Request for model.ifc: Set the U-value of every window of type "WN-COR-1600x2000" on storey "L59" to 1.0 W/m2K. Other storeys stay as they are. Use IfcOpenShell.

First a look at what the model holds.

```python
import ifcopenshell
import ifcopenshell.util.element

model = ifcopenshell.open("model.ifc")
print(model.schema)
storey = next(s for s in model.by_type("IfcBuildingStorey") if s.Name == "L59")
windows = [e for e in ifcopenshell.util.element.get_decomposition(storey) if e.is_a("IfcWindow")]
seen = {}
for e in windows:
    element_type = ifcopenshell.util.element.get_type(e)
    key = (element_type.Name if element_type != e and element_type else None, ifcopenshell.util.element.get_pset(e, "Pset_WindowCommon", "ThermalTransmittance"))
    seen[key] = seen.get(key, 0) + 1
for (name, value), count in sorted(seen.items(), key=str):
    print(count, "x", name, "|", value)
```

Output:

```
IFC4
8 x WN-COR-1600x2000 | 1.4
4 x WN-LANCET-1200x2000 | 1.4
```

```python
import ifcopenshell
import ifcopenshell.api.pset
import ifcopenshell.util.element

model = ifcopenshell.open("model.ifc")

storey = next(s for s in model.by_type("IfcBuildingStorey") if s.Name == "L59")
windows = [e for e in ifcopenshell.util.element.get_decomposition(storey) if e.is_a("IfcWindow")]

count = 0
for e in windows:
    element_type = ifcopenshell.util.element.get_type(e)
    if element_type in (None, e) or element_type.Name != "WN-COR-1600x2000":
        continue
    found = ifcopenshell.util.element.get_pset(e, "Pset_WindowCommon", should_inherit=False)
    if found:
        pset = model.by_id(found["id"])
        if len(ifcopenshell.util.element.get_elements_by_pset(pset)) > 1:
            pset = ifcopenshell.api.pset.unshare_pset(model, products=[e], pset=pset)[0]
    else:
        pset = ifcopenshell.api.pset.add_pset(model, product=e, name="Pset_WindowCommon")
    ifcopenshell.api.pset.edit_pset(model, pset=pset, properties={"ThermalTransmittance": 1.0})
    count += 1

print(count, "windows updated")

model.write("model_edited.ifc")
```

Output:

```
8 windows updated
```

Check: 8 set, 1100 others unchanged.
